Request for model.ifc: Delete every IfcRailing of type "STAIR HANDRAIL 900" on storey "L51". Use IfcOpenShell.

First a look at what the model holds.

```python
import ifcopenshell
import ifcopenshell.util.element

model = ifcopenshell.open("model.ifc")
print(model.schema)
storey = next(s for s in model.by_type("IfcBuildingStorey") if s.Name == "L51")
railings = [e for e in ifcopenshell.util.element.get_decomposition(storey) if e.is_a("IfcRailing")]
seen = {}
for e in railings:
    element_type = ifcopenshell.util.element.get_type(e)
    name = element_type.Name if element_type not in (None, e) else None
    seen[name] = seen.get(name, 0) + 1
for name, count in sorted(seen.items(), key=str):
    print(count, "x", name)
```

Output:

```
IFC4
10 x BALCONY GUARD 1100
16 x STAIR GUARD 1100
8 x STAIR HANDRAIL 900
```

```python
import ifcopenshell
import ifcopenshell.api.root
import ifcopenshell.util.element

model = ifcopenshell.open("model.ifc")

storey = next(s for s in model.by_type("IfcBuildingStorey") if s.Name == "L51")
railings = [e for e in ifcopenshell.util.element.get_decomposition(storey) if e.is_a("IfcRailing")]
targets = [e for e in railings if (t := ifcopenshell.util.element.get_type(e)) not in (None, e) and t.Name == "STAIR HANDRAIL 900"]

for e in targets:
    ifcopenshell.api.root.remove_product(model, product=e)
print(len(targets), "removed")

model.write("model_edited.ifc")
```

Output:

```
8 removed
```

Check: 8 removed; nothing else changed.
